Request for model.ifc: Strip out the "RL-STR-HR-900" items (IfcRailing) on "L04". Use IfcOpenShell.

First a look at what the model holds.

```python
import ifcopenshell
import ifcopenshell.util.element

model = ifcopenshell.open("model.ifc")
print(model.schema)
storey = next(s for s in model.by_type("IfcBuildingStorey") if s.Name == "L04")
railings = [e for e in ifcopenshell.util.element.get_decomposition(storey) if e.is_a("IfcRailing")]
seen = {}
for e in railings:
    element_type = ifcopenshell.util.element.get_type(e)
    name = element_type.Name if element_type not in (None, e) else None
    seen[name] = seen.get(name, 0) + 1
for name, count in sorted(seen.items(), key=str):
    print(count, "x", name)
```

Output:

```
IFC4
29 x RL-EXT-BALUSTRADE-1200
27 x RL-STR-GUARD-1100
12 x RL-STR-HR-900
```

```python
import ifcopenshell
import ifcopenshell.api.root
import ifcopenshell.util.element

model = ifcopenshell.open("model.ifc")

storey = next(s for s in model.by_type("IfcBuildingStorey") if s.Name == "L04")
railings = [e for e in ifcopenshell.util.element.get_decomposition(storey) if e.is_a("IfcRailing")]
targets = [e for e in railings if (t := ifcopenshell.util.element.get_type(e)) not in (None, e) and t.Name == "RL-STR-HR-900"]

for e in targets:
    ifcopenshell.api.root.remove_product(model, product=e)
print(len(targets), "removed")

model.write("model_v2.ifc")
```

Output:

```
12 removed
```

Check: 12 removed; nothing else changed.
